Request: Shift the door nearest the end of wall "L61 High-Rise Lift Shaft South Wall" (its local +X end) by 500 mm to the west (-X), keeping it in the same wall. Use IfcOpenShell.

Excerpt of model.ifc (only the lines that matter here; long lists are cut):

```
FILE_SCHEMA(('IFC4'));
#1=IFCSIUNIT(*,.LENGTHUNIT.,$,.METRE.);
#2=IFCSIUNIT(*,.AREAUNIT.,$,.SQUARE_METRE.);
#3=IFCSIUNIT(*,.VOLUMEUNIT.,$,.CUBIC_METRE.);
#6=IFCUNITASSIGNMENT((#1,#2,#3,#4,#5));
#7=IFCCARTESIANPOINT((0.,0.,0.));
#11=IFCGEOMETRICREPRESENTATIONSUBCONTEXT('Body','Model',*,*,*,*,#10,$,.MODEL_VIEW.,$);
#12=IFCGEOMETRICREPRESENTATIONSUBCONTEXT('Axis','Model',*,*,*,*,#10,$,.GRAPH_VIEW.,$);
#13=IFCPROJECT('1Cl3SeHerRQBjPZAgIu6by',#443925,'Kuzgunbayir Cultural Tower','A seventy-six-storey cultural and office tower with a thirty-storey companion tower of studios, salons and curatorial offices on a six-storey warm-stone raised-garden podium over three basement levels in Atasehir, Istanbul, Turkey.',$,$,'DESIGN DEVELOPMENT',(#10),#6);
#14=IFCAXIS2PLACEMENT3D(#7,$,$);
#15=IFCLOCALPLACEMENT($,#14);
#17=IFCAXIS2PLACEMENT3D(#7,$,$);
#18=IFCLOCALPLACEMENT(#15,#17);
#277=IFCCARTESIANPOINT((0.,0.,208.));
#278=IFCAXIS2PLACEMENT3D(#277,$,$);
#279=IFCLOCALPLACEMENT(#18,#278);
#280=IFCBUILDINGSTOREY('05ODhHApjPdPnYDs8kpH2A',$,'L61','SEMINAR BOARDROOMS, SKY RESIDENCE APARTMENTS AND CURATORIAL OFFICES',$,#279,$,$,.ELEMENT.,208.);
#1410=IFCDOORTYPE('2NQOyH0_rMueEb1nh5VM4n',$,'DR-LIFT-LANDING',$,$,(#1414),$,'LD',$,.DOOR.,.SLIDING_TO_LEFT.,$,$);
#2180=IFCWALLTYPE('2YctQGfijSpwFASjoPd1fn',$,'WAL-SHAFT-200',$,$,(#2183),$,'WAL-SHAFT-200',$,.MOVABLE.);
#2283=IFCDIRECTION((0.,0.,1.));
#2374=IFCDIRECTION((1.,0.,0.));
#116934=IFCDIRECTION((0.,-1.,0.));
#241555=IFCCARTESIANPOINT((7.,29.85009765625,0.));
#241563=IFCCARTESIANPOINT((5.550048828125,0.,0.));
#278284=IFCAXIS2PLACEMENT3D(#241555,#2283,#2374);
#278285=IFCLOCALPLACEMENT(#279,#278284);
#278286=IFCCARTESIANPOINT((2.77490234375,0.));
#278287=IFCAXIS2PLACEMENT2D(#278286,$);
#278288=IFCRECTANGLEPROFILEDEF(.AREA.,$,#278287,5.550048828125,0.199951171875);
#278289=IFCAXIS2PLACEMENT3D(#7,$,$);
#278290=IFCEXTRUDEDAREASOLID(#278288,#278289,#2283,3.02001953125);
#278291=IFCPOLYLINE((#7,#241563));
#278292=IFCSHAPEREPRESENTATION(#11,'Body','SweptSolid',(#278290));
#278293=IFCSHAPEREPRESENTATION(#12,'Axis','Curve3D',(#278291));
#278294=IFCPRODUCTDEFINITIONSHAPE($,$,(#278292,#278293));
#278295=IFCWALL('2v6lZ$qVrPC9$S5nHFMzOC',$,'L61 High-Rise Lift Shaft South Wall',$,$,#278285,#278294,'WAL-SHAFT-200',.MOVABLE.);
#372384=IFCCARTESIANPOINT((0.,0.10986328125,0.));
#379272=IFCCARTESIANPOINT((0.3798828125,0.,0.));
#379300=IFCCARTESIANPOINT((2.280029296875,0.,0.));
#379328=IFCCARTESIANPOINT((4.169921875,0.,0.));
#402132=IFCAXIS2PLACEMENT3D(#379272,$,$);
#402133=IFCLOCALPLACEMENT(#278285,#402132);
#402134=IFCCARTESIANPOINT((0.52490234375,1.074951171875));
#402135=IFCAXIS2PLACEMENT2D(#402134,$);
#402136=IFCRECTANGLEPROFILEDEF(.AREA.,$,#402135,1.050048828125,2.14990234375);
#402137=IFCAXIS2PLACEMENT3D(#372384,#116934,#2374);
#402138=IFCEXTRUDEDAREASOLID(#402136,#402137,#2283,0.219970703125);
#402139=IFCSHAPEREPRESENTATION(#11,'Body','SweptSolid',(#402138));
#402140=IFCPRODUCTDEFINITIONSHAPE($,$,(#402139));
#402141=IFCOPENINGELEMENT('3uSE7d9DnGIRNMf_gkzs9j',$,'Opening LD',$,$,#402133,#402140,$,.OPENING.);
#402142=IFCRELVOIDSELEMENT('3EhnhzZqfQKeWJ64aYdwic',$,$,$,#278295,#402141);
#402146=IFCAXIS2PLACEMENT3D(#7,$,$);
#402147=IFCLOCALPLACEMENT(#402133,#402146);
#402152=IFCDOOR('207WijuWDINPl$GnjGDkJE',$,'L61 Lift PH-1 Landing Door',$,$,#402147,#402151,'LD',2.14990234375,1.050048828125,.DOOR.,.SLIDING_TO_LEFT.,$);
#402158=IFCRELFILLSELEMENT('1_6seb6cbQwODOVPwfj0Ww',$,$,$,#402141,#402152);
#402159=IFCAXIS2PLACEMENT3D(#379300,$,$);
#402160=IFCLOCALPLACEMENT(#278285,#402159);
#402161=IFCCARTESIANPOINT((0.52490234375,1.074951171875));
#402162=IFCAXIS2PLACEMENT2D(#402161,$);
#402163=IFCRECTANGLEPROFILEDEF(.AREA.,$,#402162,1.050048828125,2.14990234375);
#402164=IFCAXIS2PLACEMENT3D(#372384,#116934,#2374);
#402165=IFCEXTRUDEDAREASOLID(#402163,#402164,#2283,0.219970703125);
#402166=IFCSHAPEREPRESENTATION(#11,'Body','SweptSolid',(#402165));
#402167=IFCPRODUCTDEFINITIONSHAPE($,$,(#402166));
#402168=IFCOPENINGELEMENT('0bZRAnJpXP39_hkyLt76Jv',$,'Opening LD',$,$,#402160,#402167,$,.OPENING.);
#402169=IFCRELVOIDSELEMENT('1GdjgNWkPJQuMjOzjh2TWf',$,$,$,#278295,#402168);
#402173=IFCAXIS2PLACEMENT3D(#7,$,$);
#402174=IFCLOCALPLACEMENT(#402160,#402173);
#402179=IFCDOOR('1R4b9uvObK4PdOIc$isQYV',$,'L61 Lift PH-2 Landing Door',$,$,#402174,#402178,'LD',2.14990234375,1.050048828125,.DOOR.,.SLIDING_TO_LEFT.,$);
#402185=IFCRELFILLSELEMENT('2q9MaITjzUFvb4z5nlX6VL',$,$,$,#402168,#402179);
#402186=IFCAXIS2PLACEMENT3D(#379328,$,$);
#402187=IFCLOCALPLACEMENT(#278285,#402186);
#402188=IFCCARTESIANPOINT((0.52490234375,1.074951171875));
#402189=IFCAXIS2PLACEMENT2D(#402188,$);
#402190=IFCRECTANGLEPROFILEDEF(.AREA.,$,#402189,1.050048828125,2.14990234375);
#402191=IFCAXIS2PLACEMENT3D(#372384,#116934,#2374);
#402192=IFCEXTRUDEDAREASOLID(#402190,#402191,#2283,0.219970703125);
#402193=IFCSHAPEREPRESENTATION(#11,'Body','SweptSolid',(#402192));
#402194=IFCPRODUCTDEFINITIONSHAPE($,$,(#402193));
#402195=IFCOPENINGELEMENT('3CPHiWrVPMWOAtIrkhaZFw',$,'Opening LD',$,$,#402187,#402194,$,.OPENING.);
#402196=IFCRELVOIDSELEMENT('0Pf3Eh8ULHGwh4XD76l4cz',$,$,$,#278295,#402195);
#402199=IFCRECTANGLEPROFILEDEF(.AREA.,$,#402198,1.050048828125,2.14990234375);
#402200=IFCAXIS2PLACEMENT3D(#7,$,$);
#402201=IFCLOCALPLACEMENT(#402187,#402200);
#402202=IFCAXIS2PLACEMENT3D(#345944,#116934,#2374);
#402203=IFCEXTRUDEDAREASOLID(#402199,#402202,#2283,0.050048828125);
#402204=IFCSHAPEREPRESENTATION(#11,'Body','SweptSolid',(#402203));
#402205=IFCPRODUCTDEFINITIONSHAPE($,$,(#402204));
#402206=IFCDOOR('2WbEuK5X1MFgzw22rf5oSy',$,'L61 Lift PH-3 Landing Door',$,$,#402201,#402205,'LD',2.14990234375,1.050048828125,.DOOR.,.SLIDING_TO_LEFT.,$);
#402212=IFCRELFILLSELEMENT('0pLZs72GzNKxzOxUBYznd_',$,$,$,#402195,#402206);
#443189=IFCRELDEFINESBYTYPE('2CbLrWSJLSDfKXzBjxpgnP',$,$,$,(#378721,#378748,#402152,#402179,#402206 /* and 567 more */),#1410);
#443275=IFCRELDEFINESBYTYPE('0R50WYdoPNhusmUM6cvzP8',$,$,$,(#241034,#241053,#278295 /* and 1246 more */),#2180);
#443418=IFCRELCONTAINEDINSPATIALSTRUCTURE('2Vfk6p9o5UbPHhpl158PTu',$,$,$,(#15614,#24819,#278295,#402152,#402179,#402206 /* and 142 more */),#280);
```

```python
import ifcopenshell
import ifcopenshell.api.geometry
import ifcopenshell.util.placement
import ifcopenshell.util.unit

model = ifcopenshell.open("model.ifc")
unit_scale = ifcopenshell.util.unit.calculate_unit_scale(model)

door = model.by_guid("2WbEuK5X1MFgzw22rf5oSy")
opening = door.FillsVoids[0].RelatingOpeningElement
wall = opening.VoidsElements[0].RelatingBuildingElement

wall_matrix = ifcopenshell.util.placement.get_local_placement(wall.ObjectPlacement)
shift = wall_matrix[:3, 0] * -0.5 / unit_scale
before = ifcopenshell.util.placement.get_local_placement(door.ObjectPlacement)[:3, 3].copy()

# The door is placed relative to its opening, so it follows when the opening moves.
matrix = ifcopenshell.util.placement.get_local_placement(opening.ObjectPlacement)
matrix[:3, 3] += shift
ifcopenshell.api.geometry.edit_object_placement(
    model, product=opening, matrix=matrix, is_si=False, should_transform_children=True
)

after = ifcopenshell.util.placement.get_local_placement(door.ObjectPlacement)[:3, 3]
print("door moved by", (after - before).round(3) + 0.0)

model.write("model-out.ifc")
```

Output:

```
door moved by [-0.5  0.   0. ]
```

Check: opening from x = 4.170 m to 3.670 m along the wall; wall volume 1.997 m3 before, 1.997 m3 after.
